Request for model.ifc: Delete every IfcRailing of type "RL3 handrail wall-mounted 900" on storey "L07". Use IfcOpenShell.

First a look at what the model holds.

```python
import ifcopenshell
import ifcopenshell.util.element

model = ifcopenshell.open("model.ifc")
print(model.schema)
storey = next(s for s in model.by_type("IfcBuildingStorey") if s.Name == "L07")
railings = [e for e in ifcopenshell.util.element.get_decomposition(storey) if e.is_a("IfcRailing")]
seen = {}
for e in railings:
    element_type = ifcopenshell.util.element.get_type(e)
    name = element_type.Name if element_type not in (None, e) else None
    seen[name] = seen.get(name, 0) + 1
for name, count in sorted(seen.items(), key=str):
    print(count, "x", name)
```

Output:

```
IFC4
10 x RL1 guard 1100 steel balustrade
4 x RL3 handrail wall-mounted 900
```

```python
import ifcopenshell
import ifcopenshell.api.root
import ifcopenshell.util.element

model = ifcopenshell.open("model.ifc")

storey = next(s for s in model.by_type("IfcBuildingStorey") if s.Name == "L07")
railings = [e for e in ifcopenshell.util.element.get_decomposition(storey) if e.is_a("IfcRailing")]
targets = [e for e in railings if (t := ifcopenshell.util.element.get_type(e)) not in (None, e) and t.Name == "RL3 handrail wall-mounted 900"]

for e in targets:
    ifcopenshell.api.root.remove_product(model, product=e)
print(len(targets), "removed")

model.write("model_edited.ifc")
```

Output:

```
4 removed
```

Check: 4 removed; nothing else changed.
